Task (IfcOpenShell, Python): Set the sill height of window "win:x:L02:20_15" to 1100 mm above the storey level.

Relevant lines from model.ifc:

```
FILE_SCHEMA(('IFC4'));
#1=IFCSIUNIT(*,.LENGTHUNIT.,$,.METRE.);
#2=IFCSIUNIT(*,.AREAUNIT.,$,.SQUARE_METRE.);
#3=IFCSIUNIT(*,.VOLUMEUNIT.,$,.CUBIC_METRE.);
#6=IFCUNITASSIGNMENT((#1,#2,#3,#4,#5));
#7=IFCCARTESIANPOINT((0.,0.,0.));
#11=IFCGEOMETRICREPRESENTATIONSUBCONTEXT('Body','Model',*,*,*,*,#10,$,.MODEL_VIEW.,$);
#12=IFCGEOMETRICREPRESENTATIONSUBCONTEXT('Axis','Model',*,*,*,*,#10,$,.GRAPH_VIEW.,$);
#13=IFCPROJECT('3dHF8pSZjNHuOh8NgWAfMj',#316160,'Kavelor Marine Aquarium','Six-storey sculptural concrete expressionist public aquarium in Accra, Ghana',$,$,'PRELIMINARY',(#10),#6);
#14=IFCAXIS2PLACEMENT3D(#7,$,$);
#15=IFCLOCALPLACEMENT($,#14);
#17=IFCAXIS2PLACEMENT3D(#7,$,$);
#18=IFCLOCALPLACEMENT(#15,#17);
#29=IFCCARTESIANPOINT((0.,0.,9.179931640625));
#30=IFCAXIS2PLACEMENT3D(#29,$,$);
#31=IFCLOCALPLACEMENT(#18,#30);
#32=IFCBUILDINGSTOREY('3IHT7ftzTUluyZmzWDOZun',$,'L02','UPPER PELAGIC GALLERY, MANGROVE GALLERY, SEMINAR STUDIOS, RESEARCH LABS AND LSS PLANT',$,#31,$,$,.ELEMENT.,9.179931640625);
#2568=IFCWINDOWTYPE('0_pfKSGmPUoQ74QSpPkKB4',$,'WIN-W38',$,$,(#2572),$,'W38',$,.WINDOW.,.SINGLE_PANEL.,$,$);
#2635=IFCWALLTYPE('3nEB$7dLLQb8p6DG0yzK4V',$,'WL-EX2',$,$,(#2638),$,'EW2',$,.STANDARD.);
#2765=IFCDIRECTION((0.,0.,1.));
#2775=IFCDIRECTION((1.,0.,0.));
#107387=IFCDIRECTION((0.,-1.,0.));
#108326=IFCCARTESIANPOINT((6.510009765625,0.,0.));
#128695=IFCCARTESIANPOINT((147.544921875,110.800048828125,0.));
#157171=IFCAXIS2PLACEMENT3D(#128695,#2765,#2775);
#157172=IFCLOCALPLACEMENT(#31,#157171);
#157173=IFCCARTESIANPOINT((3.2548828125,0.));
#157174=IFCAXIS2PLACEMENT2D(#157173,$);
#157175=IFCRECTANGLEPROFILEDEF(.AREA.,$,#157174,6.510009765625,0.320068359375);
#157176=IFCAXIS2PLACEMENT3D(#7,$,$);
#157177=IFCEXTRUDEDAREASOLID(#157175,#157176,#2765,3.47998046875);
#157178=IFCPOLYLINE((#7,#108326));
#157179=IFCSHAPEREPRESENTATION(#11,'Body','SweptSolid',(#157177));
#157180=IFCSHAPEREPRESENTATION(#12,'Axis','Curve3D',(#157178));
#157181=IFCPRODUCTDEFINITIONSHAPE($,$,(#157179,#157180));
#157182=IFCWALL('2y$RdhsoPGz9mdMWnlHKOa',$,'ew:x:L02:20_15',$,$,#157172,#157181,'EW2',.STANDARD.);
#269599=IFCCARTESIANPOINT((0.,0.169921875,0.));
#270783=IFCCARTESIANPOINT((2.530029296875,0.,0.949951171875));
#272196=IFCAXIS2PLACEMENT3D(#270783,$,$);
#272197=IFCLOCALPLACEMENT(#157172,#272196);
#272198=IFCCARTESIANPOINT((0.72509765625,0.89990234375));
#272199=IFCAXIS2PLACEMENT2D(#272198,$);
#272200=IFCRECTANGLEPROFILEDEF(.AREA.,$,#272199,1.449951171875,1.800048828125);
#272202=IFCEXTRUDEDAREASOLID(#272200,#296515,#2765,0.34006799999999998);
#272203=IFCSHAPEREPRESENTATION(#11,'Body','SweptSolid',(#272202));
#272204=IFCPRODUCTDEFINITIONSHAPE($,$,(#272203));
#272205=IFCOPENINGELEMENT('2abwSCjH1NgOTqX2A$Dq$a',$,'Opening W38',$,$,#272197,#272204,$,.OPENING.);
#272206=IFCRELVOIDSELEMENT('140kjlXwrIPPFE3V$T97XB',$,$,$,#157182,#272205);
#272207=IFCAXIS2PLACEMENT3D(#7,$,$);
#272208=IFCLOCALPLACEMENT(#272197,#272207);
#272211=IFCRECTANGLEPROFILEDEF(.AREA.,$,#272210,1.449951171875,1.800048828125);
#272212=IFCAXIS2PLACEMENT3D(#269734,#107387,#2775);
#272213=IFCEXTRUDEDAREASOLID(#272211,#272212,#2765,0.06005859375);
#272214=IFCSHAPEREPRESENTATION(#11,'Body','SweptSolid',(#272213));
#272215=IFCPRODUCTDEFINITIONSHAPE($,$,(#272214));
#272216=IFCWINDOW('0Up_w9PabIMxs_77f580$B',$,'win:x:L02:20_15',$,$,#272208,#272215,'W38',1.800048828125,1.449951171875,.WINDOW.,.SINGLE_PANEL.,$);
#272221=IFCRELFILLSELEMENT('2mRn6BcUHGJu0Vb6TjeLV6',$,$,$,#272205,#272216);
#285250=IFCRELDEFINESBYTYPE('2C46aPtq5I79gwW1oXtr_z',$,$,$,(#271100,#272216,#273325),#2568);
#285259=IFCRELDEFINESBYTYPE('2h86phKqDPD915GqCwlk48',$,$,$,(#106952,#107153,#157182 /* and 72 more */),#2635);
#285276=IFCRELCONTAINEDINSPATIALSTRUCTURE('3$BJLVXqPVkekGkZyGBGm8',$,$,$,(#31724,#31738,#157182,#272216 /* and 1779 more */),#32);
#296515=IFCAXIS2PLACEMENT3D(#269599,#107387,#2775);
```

```python
import numpy as np
import ifcopenshell
import ifcopenshell.api.geometry
import ifcopenshell.geom
import ifcopenshell.util.element
import ifcopenshell.util.placement
import ifcopenshell.util.shape
import ifcopenshell.util.unit

model = ifcopenshell.open("model.ifc")
unit_scale = ifcopenshell.util.unit.calculate_unit_scale(model)

window = model.by_guid("0Up_w9PabIMxs_77f580$B")
opening = window.FillsVoids[0].RelatingOpeningElement
storey = ifcopenshell.util.element.get_container(window, ifc_class="IfcBuildingStorey")
level = ifcopenshell.util.placement.get_local_placement(storey.ObjectPlacement)[2, 3]

# The opening's origin need not be at the sill, so measure its lowest point.
shape = ifcopenshell.geom.create_shape(ifcopenshell.geom.settings(), opening)
bottom = ifcopenshell.util.shape.get_shape_bottom_elevation(shape, shape.geometry) / unit_scale
dz = level + 1.1 - bottom

shift = np.array([0.0, 0.0, dz])
# The window is placed relative to its opening, so it follows when the opening moves.
matrix = ifcopenshell.util.placement.get_local_placement(opening.ObjectPlacement)
matrix[:3, 3] += shift
ifcopenshell.api.geometry.edit_object_placement(
    model, product=opening, matrix=matrix, is_si=False, should_transform_children=True
)

print(f"moved by {dz * unit_scale:+.3f} m")

model.write("model_rev.ifc")
```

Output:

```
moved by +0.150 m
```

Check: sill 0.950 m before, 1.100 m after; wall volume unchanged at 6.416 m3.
